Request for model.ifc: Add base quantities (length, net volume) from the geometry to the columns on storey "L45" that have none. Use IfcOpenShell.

First a look at what the model holds.

```python
import ifcopenshell
import ifcopenshell.util.element
import ifcopenshell.util.unit

model = ifcopenshell.open("model.ifc")
print(model.schema)
for unit_type in ("LENGTHUNIT", "AREAUNIT", "VOLUMEUNIT"):
    print(unit_type, ifcopenshell.util.unit.calculate_unit_scale(model, unit_type))
storey = next(s for s in model.by_type("IfcBuildingStorey") if s.Name == "L45")
columns = [e for e in ifcopenshell.util.element.get_decomposition(storey) if e.is_a("IfcColumn")]
for e in sorted(columns, key=lambda e: e.id()):
    print(e.id(), e.is_a(), e.Name, list(ifcopenshell.util.element.get_psets(e, qtos_only=True)), sep=" | ")
```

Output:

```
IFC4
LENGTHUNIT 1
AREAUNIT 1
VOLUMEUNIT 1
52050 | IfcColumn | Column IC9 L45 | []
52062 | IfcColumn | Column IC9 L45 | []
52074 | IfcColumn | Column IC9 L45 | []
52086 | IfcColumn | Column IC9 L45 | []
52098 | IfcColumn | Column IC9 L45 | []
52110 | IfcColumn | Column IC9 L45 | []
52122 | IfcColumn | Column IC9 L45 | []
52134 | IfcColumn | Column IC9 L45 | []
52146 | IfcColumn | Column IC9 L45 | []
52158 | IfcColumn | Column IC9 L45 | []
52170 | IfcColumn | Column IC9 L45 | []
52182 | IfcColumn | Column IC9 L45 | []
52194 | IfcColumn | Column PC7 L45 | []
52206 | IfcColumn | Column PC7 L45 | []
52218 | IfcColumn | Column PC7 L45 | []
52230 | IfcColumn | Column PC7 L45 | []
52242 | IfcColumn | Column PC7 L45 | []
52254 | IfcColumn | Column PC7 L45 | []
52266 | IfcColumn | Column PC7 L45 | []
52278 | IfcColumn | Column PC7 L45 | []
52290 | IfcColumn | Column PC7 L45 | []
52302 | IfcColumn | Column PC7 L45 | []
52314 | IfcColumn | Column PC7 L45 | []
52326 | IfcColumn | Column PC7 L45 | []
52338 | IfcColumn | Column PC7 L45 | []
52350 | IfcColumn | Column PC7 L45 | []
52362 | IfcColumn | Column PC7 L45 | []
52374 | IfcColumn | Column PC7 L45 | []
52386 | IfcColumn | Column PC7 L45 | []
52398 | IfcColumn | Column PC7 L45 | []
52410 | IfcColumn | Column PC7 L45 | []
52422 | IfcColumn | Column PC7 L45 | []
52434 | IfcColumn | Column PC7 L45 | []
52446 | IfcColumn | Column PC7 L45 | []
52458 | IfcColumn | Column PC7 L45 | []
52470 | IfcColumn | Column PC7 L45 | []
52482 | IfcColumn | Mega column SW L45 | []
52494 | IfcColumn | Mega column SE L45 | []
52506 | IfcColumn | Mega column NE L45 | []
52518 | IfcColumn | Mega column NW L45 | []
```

```python
import ifcopenshell
import ifcopenshell.api.pset
import ifcopenshell.geom
import ifcopenshell.util.element
import ifcopenshell.util.shape
import ifcopenshell.util.unit

model = ifcopenshell.open("model.ifc")
unit_scale = ifcopenshell.util.unit.calculate_unit_scale(model)
volume_scale = ifcopenshell.util.unit.calculate_unit_scale(model, "VOLUMEUNIT")
settings = ifcopenshell.geom.settings()

storey = next(s for s in model.by_type("IfcBuildingStorey") if s.Name == "L45")
columns = [e for e in ifcopenshell.util.element.get_decomposition(storey) if e.is_a("IfcColumn")]

for e in sorted(columns, key=lambda e: e.id()):
    if ifcopenshell.util.element.get_psets(e, qtos_only=True, should_inherit=False):
        continue
    # Geometry comes back in metres, in the element's own axes.
    shape = ifcopenshell.geom.create_shape(settings, e)
    values = {
        "Length": ifcopenshell.util.shape.get_z(shape.geometry) / unit_scale,
        "NetVolume": ifcopenshell.util.shape.get_volume(shape.geometry) / volume_scale,
    }
    qto = ifcopenshell.api.pset.add_qto(model, product=e, name="Qto_ColumnBaseQuantities")
    ifcopenshell.api.pset.edit_qto(model, qto=qto, properties=values)
    print(e.id(), {k: round(v, 3) for k, v in values.items()})

model.write("model_updated.ifc")
```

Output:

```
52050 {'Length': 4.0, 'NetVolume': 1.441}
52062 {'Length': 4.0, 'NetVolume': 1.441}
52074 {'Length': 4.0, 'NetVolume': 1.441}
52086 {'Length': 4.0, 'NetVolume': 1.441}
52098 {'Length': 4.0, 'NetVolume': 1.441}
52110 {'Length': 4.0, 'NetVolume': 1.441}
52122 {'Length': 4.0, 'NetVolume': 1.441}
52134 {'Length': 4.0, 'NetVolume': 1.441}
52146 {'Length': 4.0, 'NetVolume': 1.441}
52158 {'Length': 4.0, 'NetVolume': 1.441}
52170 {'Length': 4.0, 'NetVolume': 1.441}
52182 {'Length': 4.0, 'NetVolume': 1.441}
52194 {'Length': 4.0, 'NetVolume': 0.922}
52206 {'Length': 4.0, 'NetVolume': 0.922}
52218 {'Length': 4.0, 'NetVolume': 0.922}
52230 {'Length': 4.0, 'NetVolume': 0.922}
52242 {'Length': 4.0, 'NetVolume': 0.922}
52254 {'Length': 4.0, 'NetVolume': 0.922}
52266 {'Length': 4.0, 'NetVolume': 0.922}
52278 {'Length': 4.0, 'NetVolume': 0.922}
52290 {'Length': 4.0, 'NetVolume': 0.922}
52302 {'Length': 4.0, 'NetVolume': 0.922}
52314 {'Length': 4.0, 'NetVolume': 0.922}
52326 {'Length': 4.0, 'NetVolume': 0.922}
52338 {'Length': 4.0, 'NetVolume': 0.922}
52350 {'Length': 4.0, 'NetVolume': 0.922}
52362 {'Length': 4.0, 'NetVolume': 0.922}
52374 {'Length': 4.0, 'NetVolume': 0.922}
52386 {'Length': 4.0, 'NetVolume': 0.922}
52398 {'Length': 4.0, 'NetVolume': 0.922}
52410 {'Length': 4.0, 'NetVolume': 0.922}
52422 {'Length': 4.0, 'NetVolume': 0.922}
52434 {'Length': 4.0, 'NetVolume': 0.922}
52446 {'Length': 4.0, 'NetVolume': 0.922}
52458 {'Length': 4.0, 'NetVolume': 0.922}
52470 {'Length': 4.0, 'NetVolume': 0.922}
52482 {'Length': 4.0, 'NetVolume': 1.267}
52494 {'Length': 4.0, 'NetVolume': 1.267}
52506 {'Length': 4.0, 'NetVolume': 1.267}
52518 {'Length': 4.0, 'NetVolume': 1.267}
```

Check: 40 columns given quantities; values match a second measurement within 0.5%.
